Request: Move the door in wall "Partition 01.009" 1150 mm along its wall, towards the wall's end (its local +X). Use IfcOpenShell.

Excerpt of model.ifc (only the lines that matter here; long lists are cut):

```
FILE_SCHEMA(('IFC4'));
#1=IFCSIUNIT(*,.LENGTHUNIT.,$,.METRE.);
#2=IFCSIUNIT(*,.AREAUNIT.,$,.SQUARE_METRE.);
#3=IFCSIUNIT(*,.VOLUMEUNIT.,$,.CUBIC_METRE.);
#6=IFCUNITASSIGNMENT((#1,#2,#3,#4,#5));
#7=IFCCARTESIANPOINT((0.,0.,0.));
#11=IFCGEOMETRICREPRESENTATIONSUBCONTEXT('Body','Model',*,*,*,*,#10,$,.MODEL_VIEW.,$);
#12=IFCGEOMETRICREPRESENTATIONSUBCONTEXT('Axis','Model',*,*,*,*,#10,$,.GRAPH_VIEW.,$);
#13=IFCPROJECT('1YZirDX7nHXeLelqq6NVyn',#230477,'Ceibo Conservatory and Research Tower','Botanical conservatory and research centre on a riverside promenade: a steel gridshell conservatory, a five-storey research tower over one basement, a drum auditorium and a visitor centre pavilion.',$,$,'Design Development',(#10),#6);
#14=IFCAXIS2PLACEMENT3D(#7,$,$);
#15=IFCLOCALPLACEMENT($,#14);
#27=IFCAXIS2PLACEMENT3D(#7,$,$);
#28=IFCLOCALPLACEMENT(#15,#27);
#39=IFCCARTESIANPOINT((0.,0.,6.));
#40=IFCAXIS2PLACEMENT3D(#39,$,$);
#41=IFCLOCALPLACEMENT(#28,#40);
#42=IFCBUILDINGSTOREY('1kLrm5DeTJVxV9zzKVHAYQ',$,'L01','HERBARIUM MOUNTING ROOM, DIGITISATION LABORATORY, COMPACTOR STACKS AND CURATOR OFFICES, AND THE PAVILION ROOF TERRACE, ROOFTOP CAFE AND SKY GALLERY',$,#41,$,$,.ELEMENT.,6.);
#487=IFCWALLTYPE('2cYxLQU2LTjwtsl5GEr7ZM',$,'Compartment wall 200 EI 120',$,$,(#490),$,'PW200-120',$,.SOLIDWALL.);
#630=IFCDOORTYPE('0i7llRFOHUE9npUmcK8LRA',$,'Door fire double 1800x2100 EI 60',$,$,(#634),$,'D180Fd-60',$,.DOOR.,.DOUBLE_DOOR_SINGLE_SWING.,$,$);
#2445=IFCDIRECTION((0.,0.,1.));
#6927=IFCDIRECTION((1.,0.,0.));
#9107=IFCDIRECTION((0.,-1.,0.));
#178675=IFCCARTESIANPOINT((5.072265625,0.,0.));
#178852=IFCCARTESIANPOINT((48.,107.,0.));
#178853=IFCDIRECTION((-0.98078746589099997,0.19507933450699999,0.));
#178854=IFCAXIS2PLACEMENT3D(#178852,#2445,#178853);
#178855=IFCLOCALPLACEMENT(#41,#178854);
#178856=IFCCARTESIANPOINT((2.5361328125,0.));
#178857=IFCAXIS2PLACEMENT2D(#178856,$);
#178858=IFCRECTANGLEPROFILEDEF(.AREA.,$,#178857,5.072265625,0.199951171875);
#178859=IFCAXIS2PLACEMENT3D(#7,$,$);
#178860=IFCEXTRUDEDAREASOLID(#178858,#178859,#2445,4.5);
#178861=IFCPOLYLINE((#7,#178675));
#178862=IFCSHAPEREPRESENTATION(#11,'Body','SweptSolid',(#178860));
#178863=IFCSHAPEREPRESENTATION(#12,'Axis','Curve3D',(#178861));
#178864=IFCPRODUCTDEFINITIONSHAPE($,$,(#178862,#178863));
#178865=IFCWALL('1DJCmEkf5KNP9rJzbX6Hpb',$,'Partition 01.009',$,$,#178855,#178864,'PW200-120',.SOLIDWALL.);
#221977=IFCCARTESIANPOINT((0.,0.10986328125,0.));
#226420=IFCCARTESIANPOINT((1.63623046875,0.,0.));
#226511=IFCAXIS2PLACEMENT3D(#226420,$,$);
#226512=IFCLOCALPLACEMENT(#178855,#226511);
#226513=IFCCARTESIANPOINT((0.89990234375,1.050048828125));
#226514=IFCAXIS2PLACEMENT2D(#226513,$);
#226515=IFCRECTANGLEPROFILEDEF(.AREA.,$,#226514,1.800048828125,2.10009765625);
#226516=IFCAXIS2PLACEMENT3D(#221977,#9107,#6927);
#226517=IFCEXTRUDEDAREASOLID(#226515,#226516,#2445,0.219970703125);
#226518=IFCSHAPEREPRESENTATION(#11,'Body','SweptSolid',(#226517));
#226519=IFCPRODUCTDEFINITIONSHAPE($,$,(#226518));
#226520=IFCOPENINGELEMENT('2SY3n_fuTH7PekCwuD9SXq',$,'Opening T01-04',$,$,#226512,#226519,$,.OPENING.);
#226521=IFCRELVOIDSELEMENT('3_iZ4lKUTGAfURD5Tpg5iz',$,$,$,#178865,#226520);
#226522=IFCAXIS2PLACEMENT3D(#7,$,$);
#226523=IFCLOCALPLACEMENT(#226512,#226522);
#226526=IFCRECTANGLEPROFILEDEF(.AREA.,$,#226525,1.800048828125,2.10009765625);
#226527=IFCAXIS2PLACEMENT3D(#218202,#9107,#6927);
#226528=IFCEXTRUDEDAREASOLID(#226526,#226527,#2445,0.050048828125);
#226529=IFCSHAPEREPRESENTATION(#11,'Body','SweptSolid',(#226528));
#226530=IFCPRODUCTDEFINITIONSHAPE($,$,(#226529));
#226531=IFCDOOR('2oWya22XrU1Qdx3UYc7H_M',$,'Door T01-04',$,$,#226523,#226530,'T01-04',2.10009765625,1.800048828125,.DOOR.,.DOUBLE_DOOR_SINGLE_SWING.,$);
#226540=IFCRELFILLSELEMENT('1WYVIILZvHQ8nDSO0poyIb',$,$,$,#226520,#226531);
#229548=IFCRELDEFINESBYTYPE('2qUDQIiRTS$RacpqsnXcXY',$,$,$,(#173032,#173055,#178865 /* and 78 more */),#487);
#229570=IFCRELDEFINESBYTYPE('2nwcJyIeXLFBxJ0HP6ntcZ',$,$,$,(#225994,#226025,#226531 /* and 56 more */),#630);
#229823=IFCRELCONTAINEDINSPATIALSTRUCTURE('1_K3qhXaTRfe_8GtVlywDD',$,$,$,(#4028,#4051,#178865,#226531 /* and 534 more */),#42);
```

```python
import ifcopenshell
import ifcopenshell.api.geometry
import ifcopenshell.util.placement

model = ifcopenshell.open("model.ifc")

door = model.by_guid("2oWya22XrU1Qdx3UYc7H_M")
opening = door.FillsVoids[0].RelatingOpeningElement
wall = opening.VoidsElements[0].RelatingBuildingElement

wall_matrix = ifcopenshell.util.placement.get_local_placement(wall.ObjectPlacement)
shift = wall_matrix[:3, 0] * 1.15
before = ifcopenshell.util.placement.get_local_placement(door.ObjectPlacement)[:3, 3].copy()

# The door is placed relative to its opening, so it follows when the opening moves.
matrix = ifcopenshell.util.placement.get_local_placement(opening.ObjectPlacement)
matrix[:3, 3] += shift
ifcopenshell.api.geometry.edit_object_placement(
    model, product=opening, matrix=matrix, is_si=False, should_transform_children=True
)

after = ifcopenshell.util.placement.get_local_placement(door.ObjectPlacement)[:3, 3]
print("door moved by", (after - before).round(3) + 0.0)

model.write("model_v2.ifc")
```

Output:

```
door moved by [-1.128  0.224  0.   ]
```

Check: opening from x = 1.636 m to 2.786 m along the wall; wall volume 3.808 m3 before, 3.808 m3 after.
